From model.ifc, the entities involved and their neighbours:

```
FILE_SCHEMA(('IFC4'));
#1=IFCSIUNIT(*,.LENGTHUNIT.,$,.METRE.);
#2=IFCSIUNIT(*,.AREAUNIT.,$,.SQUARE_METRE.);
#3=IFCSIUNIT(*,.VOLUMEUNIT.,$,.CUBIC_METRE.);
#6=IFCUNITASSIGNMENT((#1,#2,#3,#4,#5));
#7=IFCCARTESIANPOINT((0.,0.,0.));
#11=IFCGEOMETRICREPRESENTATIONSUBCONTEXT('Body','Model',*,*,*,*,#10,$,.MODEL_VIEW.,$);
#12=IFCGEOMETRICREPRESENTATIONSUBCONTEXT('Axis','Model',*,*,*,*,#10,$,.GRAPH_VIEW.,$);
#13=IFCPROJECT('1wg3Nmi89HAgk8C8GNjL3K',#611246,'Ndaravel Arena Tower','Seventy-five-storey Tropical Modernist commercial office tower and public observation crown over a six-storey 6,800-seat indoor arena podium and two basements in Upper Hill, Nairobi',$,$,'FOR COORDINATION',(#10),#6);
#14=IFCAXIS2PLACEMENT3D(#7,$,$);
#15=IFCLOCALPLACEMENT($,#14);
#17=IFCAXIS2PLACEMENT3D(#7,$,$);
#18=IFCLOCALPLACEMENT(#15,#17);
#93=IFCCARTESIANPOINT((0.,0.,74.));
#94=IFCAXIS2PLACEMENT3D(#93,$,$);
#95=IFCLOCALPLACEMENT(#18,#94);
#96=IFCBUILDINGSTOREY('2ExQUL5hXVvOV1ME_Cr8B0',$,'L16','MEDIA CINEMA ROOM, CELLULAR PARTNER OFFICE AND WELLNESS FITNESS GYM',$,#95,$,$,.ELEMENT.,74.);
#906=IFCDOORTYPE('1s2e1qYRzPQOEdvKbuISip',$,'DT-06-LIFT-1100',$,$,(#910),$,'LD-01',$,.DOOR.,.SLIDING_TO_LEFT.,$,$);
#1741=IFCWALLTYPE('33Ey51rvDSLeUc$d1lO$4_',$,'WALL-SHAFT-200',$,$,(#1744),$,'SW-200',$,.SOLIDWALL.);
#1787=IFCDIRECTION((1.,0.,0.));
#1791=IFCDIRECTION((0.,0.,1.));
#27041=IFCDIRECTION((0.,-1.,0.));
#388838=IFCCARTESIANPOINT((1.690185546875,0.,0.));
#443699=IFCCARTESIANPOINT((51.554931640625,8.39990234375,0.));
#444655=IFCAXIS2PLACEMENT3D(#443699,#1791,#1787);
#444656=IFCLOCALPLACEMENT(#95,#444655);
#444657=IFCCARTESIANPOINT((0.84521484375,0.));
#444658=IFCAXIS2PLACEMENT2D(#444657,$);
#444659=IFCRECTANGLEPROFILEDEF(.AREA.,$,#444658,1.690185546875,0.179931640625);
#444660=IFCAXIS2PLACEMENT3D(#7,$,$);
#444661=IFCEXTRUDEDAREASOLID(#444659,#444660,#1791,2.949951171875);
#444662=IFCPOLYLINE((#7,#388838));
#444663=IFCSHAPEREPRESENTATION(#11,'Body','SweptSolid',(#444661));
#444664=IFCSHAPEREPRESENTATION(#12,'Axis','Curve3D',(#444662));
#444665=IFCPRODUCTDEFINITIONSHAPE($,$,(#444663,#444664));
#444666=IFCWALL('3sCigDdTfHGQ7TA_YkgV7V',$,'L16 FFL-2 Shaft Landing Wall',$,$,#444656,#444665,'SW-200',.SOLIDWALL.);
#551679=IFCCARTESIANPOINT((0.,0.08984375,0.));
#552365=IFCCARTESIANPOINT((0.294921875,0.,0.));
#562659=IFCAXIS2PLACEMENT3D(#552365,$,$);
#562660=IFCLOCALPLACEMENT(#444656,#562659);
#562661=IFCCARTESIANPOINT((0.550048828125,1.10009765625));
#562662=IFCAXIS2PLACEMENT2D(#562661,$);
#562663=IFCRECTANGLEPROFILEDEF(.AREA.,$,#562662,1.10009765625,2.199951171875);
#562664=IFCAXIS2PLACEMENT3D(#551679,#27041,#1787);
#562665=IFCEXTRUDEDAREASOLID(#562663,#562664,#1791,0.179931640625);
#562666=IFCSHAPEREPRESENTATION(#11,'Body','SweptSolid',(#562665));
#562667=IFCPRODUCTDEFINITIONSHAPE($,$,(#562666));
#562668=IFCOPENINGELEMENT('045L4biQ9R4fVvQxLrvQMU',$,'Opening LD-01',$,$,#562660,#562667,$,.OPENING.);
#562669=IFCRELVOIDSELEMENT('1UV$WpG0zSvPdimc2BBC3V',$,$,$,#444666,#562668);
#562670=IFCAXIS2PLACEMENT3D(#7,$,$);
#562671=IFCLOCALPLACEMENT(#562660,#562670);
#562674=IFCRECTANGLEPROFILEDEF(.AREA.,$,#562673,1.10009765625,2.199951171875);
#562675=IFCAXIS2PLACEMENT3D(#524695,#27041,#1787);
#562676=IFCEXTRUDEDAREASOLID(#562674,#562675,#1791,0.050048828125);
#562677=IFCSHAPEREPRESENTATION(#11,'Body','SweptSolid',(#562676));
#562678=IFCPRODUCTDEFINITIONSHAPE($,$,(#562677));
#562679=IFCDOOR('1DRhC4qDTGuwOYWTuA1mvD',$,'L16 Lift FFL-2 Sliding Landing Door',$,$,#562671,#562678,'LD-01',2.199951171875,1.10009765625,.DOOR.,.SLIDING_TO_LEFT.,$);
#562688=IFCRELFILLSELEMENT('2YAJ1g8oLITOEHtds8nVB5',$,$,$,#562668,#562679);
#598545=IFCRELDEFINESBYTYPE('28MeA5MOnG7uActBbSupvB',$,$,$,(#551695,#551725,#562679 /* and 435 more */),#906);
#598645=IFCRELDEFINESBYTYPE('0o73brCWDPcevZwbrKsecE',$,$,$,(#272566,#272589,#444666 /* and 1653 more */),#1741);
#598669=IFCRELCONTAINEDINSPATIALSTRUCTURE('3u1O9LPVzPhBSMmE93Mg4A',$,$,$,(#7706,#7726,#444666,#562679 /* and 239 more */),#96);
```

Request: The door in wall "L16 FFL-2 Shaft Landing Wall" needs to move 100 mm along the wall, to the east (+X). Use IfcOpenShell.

```python
import ifcopenshell
import ifcopenshell.api.geometry
import ifcopenshell.util.placement
import ifcopenshell.util.unit

model = ifcopenshell.open("model.ifc")
unit_scale = ifcopenshell.util.unit.calculate_unit_scale(model)

door = model.by_id(562679)
opening = door.FillsVoids[0].RelatingOpeningElement
wall = opening.VoidsElements[0].RelatingBuildingElement

wall_matrix = ifcopenshell.util.placement.get_local_placement(wall.ObjectPlacement)
shift = wall_matrix[:3, 0] * 0.1 / unit_scale
before = ifcopenshell.util.placement.get_local_placement(door.ObjectPlacement)[:3, 3].copy()

# The door is placed relative to its opening, so it follows when the opening moves.
matrix = ifcopenshell.util.placement.get_local_placement(opening.ObjectPlacement)
matrix[:3, 3] += shift
ifcopenshell.api.geometry.edit_object_placement(
    model, product=opening, matrix=matrix, is_si=False, should_transform_children=True
)

after = ifcopenshell.util.placement.get_local_placement(door.ObjectPlacement)[:3, 3]
print("door moved by", (after - before).round(3) + 0.0)

model.write("model_edited.ifc")
```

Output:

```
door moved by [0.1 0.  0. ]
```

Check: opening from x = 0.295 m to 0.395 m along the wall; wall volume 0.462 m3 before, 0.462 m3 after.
